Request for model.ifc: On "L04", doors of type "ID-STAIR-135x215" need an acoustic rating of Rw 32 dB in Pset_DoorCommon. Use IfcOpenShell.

First a look at what the model holds.

```python
import ifcopenshell
import ifcopenshell.util.element

model = ifcopenshell.open("model.ifc")
print(model.schema)
storey = next(s for s in model.by_type("IfcBuildingStorey") if s.Name == "L04")
doors = [e for e in ifcopenshell.util.element.get_decomposition(storey) if e.is_a("IfcDoor")]
seen = {}
for e in doors:
    element_type = ifcopenshell.util.element.get_type(e)
    key = (element_type.Name if element_type != e and element_type else None, ifcopenshell.util.element.get_pset(e, "Pset_DoorCommon", "AcousticRating"))
    seen[key] = seen.get(key, 0) + 1
for (name, value), count in sorted(seen.items(), key=str):
    print(count, "x", name, "|", value)
```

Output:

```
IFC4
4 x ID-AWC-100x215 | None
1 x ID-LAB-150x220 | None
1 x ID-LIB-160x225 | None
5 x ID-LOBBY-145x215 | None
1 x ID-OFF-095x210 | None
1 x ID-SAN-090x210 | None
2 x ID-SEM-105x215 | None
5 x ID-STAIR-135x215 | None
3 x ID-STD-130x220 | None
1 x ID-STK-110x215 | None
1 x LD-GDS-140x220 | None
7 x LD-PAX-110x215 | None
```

```python
import ifcopenshell
import ifcopenshell.api.pset
import ifcopenshell.util.element

model = ifcopenshell.open("model.ifc")

storey = next(s for s in model.by_type("IfcBuildingStorey") if s.Name == "L04")
doors = [e for e in ifcopenshell.util.element.get_decomposition(storey) if e.is_a("IfcDoor")]

count = 0
for e in doors:
    element_type = ifcopenshell.util.element.get_type(e)
    if element_type in (None, e) or element_type.Name != "ID-STAIR-135x215":
        continue
    # add_pset returns the element's existing set when there is one.
    pset = ifcopenshell.api.pset.add_pset(model, product=e, name="Pset_DoorCommon")
    ifcopenshell.api.pset.edit_pset(model, pset=pset, properties={"AcousticRating": "Rw 32 dB"})
    count += 1

print(count, "doors updated")

model.write("model_rev.ifc")
```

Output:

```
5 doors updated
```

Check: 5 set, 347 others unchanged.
